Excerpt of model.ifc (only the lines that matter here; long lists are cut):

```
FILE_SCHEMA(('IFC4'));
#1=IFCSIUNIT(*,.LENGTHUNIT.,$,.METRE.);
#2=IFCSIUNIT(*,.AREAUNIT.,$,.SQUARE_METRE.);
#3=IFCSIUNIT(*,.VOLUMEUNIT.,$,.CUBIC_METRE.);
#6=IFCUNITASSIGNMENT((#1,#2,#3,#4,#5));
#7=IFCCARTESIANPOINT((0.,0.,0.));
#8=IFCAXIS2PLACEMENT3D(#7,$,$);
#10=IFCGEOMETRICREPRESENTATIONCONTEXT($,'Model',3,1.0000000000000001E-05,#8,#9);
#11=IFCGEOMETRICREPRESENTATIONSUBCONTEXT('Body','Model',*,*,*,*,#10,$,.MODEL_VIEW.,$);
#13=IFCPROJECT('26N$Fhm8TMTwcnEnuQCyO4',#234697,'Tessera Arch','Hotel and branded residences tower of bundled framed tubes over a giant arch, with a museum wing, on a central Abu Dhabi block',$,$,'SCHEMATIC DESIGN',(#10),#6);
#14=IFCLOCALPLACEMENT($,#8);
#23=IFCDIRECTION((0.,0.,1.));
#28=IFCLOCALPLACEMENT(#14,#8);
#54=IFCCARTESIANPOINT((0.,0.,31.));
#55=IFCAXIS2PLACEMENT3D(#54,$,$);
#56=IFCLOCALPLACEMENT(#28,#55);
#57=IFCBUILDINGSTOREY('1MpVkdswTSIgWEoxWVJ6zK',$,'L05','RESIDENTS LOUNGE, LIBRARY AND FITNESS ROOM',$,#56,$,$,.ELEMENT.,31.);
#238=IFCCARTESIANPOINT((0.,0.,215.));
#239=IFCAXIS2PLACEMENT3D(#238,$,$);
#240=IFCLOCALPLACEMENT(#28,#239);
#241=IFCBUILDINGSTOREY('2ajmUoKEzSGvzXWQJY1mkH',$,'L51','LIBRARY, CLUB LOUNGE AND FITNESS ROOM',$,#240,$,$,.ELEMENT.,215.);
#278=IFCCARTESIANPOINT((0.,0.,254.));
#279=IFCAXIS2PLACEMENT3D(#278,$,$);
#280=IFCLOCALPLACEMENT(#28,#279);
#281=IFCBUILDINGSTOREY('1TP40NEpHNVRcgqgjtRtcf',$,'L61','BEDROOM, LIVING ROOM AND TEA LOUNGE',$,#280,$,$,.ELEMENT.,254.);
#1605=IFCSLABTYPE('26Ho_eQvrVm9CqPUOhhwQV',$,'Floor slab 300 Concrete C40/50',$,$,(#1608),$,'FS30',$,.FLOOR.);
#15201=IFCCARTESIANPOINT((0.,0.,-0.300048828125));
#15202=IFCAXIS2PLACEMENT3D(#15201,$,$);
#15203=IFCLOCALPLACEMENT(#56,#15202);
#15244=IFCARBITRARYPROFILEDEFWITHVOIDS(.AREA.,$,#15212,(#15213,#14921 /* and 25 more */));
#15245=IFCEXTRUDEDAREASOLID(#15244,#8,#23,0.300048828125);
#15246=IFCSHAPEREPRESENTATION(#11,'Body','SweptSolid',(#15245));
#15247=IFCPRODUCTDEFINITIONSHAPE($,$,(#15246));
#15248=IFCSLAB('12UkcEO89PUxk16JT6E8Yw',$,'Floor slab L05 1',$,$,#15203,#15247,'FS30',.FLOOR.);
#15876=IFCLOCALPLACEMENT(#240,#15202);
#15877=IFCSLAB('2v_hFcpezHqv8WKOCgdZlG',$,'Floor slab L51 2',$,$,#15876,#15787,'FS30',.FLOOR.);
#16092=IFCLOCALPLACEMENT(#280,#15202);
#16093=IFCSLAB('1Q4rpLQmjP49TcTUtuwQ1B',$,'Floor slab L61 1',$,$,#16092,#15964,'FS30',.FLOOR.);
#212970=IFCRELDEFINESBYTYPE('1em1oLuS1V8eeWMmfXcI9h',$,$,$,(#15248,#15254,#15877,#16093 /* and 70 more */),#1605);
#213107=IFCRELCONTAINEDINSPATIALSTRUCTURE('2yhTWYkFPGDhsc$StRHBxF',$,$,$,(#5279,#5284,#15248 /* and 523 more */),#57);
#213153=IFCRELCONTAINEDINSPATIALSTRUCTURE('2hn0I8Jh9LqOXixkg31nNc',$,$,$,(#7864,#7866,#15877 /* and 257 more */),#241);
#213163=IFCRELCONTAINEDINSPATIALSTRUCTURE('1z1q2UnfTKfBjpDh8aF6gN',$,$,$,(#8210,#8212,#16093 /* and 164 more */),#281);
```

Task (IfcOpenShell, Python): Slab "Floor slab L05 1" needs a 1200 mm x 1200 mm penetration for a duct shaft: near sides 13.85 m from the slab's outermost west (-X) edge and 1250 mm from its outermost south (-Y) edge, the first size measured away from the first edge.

```python
import numpy as np
import ifcopenshell
import ifcopenshell.api.feature
import ifcopenshell.api.geometry
import ifcopenshell.api.root
import ifcopenshell.geom
import ifcopenshell.util.placement
import ifcopenshell.util.representation
import ifcopenshell.util.shape
import ifcopenshell.util.unit

model = ifcopenshell.open("model.ifc")
unit_scale = ifcopenshell.util.unit.calculate_unit_scale(model)
settings = ifcopenshell.geom.settings()


def volume(element):
    """Net volume in cubic metres, openings subtracted."""
    shape = ifcopenshell.geom.create_shape(settings, element)
    return ifcopenshell.util.shape.get_volume(shape.geometry)


slab = model.by_id(15248)
before = volume(slab)

# Extent in the slab's own axes, in metres. The edges named are its -X and -Y sides.
slab_shape = ifcopenshell.geom.create_shape(settings, slab)
vertices = ifcopenshell.util.shape.get_vertices(slab_shape.geometry)
x_min, y_min, bottom = vertices.min(axis=0)
top = vertices[:, 2].max()

opening = ifcopenshell.api.root.create_entity(model, ifc_class="IfcOpeningElement", name="Duct shaft opening", predefined_type="OPENING")
context = ifcopenshell.util.representation.get_context(model, "Model", "Body", "MODEL_VIEW")
width, depth = 1.2, 1.2
outline = [(0.0, 0.0), (width, 0.0), (width, depth), (0.0, depth), (0.0, 0.0)]
# Overshoot both faces by 50 mm so the cut is clean.
shape = ifcopenshell.api.geometry.add_slab_representation(
    model, context=context, depth=top - bottom + 0.1, polyline=outline
)
ifcopenshell.api.geometry.assign_representation(model, product=opening, representation=shape)

matrix = ifcopenshell.util.placement.get_local_placement(slab.ObjectPlacement)
matrix[:, 3] = matrix @ np.append(np.array([x_min + 13.85, y_min + 1.25, bottom - 0.05]) / unit_scale, 1.0)
ifcopenshell.api.geometry.edit_object_placement(model, product=opening, matrix=matrix, is_si=False)
ifcopenshell.api.feature.add_feature(model, feature=opening, element=slab)

after = volume(slab)

print(f"slab volume {before:.3f} -> {after:.3f} m3")

model.write("model_edited.ifc")
```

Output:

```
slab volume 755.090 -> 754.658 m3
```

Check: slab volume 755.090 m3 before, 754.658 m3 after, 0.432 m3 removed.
